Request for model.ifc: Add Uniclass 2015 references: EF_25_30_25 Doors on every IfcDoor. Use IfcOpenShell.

First a look at what the model holds.

```python
import ifcopenshell

model = ifcopenshell.open("model.ifc")
print(model.schema)
print("classifications:", [c.Name for c in model.by_type("IfcClassification")])
for ifc_class in ("IfcDoor", "IfcRoof", "IfcStair", "IfcWall", "IfcWindow"):
    print(ifc_class, len(model.by_type(ifc_class)))
```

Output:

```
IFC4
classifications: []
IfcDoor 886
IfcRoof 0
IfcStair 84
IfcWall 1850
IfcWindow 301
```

```python
import ifcopenshell
import ifcopenshell.api.classification

model = ifcopenshell.open("model.ifc")

system = ifcopenshell.api.classification.add_classification(model, classification="Uniclass 2015")

codes = {
    "IfcDoor": ("EF_25_30_25", "Doors"),
}
for ifc_class, (code, name) in codes.items():
    products = model.by_type(ifc_class)
    ifcopenshell.api.classification.add_reference(
        model, products=products, classification=system, identification=code, name=name
    )
    print(code, len(products))

model.write("model_rev.ifc")
```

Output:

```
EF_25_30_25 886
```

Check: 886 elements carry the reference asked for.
